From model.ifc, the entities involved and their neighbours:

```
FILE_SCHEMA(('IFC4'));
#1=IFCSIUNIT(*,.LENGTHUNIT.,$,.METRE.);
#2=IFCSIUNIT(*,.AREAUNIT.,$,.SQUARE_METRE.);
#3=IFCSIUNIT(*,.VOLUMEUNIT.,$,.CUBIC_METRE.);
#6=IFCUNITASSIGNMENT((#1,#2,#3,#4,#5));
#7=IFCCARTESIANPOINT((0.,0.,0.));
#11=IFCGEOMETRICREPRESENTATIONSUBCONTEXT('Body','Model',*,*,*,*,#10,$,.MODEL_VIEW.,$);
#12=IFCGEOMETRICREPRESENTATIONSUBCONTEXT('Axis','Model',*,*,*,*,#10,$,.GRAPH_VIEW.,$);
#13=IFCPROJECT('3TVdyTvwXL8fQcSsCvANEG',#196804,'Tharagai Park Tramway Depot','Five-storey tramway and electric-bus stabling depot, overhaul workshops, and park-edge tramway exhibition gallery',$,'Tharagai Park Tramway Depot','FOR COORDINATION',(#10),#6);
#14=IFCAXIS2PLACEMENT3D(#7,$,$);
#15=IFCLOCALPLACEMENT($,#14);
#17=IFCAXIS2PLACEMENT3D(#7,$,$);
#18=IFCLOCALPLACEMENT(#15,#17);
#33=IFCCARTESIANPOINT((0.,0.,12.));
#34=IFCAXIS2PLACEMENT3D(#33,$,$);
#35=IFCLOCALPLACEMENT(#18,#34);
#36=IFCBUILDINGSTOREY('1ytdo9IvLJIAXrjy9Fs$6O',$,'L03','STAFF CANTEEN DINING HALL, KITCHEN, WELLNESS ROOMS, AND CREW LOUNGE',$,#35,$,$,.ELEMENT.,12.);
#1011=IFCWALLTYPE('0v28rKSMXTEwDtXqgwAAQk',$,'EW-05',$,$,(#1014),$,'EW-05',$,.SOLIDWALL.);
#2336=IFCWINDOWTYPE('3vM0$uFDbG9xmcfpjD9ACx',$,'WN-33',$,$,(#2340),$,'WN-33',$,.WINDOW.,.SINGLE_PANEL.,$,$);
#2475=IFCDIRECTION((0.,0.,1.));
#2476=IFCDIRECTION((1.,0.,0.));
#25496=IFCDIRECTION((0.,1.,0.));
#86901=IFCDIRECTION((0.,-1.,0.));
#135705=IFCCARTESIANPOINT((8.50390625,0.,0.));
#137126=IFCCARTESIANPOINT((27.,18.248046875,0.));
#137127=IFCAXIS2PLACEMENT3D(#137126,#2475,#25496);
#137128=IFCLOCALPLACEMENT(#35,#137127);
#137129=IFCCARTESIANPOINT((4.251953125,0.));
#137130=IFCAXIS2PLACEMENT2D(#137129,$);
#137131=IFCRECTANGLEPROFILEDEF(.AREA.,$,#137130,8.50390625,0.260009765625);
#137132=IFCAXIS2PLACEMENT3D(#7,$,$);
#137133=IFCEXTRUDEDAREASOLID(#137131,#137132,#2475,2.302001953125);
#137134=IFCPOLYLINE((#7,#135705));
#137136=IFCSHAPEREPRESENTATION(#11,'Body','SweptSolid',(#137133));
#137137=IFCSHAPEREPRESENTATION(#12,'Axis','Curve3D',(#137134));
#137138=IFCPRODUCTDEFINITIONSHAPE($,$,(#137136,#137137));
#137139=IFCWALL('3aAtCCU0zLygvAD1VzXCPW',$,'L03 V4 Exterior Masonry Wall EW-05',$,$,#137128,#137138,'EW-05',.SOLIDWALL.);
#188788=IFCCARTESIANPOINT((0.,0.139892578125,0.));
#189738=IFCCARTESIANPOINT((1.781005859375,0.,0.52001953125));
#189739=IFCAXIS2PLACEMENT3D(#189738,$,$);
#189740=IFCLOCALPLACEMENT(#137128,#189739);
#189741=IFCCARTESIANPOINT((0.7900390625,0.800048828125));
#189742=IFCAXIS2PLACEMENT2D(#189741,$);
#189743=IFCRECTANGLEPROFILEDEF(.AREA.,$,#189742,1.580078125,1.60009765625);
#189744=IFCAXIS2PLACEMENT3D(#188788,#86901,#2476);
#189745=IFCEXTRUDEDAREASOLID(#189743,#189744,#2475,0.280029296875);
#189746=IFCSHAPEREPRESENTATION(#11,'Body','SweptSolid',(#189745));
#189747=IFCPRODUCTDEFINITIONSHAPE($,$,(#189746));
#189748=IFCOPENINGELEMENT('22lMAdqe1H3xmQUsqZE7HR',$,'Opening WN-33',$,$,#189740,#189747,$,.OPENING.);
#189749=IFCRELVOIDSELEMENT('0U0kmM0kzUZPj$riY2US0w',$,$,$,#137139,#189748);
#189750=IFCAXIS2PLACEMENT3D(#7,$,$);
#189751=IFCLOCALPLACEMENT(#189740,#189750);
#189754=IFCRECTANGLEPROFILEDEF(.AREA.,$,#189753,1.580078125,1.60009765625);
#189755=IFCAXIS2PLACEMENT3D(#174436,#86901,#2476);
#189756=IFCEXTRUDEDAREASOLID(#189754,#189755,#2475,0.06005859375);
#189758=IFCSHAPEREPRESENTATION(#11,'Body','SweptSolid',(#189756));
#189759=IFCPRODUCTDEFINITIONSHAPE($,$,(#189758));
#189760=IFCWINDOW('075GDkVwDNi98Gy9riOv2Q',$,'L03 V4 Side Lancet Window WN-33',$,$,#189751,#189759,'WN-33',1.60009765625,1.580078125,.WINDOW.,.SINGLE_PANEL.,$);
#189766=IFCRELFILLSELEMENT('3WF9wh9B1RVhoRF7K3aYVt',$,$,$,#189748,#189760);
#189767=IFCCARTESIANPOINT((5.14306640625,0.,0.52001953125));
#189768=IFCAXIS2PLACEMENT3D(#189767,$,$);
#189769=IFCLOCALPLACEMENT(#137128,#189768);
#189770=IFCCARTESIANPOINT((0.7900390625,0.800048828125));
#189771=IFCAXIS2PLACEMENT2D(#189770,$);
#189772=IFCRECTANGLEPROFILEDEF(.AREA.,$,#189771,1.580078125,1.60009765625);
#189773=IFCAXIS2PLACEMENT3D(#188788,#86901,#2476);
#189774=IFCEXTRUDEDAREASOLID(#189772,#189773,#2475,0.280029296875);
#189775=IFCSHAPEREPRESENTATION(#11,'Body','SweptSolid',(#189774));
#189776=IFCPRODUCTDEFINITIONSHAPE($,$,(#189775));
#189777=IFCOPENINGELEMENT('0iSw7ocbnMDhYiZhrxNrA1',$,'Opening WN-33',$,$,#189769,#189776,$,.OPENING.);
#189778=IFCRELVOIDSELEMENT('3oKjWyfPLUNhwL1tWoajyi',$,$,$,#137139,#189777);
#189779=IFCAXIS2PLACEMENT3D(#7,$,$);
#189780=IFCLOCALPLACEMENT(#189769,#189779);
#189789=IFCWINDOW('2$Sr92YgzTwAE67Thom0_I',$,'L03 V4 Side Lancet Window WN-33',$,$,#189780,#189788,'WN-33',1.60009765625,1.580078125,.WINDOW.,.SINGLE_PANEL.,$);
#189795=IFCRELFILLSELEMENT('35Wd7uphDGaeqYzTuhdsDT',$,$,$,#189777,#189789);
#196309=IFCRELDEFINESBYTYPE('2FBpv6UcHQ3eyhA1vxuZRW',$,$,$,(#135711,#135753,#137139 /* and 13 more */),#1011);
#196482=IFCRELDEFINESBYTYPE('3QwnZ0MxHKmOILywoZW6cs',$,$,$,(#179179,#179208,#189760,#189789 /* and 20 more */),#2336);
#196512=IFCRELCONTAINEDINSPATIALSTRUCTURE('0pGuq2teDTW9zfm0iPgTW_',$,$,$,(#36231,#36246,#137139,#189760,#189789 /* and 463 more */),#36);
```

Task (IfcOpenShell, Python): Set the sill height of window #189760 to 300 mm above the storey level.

```python
import numpy as np
import ifcopenshell
import ifcopenshell.api.geometry
import ifcopenshell.geom
import ifcopenshell.util.element
import ifcopenshell.util.placement
import ifcopenshell.util.shape
import ifcopenshell.util.unit

model = ifcopenshell.open("model.ifc")
unit_scale = ifcopenshell.util.unit.calculate_unit_scale(model)

window = model.by_id(189760)
opening = window.FillsVoids[0].RelatingOpeningElement
storey = ifcopenshell.util.element.get_container(window, ifc_class="IfcBuildingStorey")
level = ifcopenshell.util.placement.get_local_placement(storey.ObjectPlacement)[2, 3]

# The opening's origin need not be at the sill, so measure its lowest point.
shape = ifcopenshell.geom.create_shape(ifcopenshell.geom.settings(), opening)
bottom = ifcopenshell.util.shape.get_shape_bottom_elevation(shape, shape.geometry) / unit_scale
dz = level + 0.3 / unit_scale - bottom

shift = np.array([0.0, 0.0, dz])
# The window is placed relative to its opening, so it follows when the opening moves.
matrix = ifcopenshell.util.placement.get_local_placement(opening.ObjectPlacement)
matrix[:3, 3] += shift
ifcopenshell.api.geometry.edit_object_placement(
    model, product=opening, matrix=matrix, is_si=False, should_transform_children=True
)

print(f"moved by {dz * unit_scale:+.3f} m")

model.write("model_v2.ifc")
```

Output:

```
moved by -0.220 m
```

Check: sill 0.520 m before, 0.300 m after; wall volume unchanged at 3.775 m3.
